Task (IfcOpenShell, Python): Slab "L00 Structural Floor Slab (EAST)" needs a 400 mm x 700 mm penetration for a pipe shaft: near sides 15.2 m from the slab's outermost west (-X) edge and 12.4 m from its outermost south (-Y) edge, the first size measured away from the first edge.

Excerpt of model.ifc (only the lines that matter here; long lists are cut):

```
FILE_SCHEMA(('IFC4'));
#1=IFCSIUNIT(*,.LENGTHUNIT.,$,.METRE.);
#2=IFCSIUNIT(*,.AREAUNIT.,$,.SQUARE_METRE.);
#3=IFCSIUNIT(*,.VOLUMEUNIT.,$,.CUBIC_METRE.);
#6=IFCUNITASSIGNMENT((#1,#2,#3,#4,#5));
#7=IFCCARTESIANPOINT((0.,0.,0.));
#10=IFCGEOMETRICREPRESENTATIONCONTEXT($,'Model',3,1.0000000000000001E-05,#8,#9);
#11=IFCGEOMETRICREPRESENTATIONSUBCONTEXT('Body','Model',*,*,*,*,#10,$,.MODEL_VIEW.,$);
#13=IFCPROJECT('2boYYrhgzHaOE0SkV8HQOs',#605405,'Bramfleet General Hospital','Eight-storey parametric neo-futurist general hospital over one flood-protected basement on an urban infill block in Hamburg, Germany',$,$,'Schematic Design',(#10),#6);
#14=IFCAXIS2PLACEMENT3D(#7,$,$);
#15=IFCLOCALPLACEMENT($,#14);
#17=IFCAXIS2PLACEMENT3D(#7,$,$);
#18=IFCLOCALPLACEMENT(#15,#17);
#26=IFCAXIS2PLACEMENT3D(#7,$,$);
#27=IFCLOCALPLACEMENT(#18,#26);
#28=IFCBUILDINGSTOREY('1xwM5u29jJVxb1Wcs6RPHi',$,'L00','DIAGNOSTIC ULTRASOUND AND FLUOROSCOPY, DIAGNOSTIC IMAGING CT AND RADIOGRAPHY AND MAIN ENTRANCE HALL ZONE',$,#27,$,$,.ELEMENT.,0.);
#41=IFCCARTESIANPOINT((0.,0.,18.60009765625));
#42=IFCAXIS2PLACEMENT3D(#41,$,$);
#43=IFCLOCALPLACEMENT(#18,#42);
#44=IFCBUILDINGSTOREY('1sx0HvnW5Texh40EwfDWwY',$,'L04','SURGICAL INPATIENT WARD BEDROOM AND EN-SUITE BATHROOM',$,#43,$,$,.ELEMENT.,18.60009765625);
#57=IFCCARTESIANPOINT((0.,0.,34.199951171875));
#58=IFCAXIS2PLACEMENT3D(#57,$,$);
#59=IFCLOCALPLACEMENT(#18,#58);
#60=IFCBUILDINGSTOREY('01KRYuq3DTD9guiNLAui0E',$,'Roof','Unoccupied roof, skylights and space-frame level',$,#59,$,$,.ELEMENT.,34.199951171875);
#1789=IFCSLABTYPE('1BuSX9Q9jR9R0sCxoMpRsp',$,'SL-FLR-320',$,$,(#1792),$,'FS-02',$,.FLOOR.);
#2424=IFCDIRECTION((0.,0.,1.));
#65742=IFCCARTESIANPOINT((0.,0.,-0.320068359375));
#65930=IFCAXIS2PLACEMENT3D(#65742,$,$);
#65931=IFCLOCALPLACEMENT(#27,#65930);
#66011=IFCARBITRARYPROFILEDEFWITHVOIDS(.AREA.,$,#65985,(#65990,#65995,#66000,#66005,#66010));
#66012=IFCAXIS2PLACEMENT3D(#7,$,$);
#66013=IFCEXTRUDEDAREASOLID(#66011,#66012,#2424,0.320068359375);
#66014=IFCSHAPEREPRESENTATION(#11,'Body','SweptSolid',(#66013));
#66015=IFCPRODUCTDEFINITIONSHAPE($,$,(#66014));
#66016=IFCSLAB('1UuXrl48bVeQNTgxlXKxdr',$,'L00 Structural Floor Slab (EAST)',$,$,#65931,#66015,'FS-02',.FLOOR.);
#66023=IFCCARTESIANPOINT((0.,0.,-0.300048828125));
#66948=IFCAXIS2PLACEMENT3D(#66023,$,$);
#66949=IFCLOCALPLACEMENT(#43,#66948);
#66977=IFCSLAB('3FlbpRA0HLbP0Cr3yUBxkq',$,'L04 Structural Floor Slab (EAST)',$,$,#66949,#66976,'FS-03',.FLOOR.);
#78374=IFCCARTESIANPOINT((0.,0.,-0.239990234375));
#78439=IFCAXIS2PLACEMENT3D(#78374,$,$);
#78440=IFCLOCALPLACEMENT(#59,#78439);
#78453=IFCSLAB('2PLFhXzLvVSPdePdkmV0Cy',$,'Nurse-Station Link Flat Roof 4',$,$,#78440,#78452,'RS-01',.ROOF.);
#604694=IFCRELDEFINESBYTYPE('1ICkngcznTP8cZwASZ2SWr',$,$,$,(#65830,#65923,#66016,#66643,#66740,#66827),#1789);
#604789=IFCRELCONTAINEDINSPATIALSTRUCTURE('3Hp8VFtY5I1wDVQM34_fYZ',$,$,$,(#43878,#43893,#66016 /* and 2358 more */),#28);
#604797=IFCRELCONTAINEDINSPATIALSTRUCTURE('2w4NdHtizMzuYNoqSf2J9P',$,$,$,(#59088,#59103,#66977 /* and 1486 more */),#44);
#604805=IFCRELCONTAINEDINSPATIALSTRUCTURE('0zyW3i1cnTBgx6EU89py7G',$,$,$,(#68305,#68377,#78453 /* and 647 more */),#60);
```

```python
import numpy as np
import ifcopenshell
import ifcopenshell.api.feature
import ifcopenshell.api.geometry
import ifcopenshell.api.root
import ifcopenshell.geom
import ifcopenshell.util.placement
import ifcopenshell.util.representation
import ifcopenshell.util.shape
import ifcopenshell.util.unit

model = ifcopenshell.open("model.ifc")
unit_scale = ifcopenshell.util.unit.calculate_unit_scale(model)
settings = ifcopenshell.geom.settings()


def volume(element):
    """Net volume in cubic metres, openings subtracted."""
    shape = ifcopenshell.geom.create_shape(settings, element)
    return ifcopenshell.util.shape.get_volume(shape.geometry)


slab = model.by_id(66016)
before = volume(slab)

# Extent in the slab's own axes, in metres. The edges named are its -X and -Y sides.
slab_shape = ifcopenshell.geom.create_shape(settings, slab)
vertices = ifcopenshell.util.shape.get_vertices(slab_shape.geometry)
x_min, y_min, bottom = vertices.min(axis=0)
top = vertices[:, 2].max()

opening = ifcopenshell.api.root.create_entity(model, ifc_class="IfcOpeningElement", name="Pipe shaft opening", predefined_type="OPENING")
context = ifcopenshell.util.representation.get_context(model, "Model", "Body", "MODEL_VIEW")
width, depth = 0.4, 0.7
outline = [(0.0, 0.0), (width, 0.0), (width, depth), (0.0, depth), (0.0, 0.0)]
# Overshoot both faces by 50 mm so the cut is clean.
shape = ifcopenshell.api.geometry.add_slab_representation(
    model, context=context, depth=top - bottom + 0.1, polyline=outline
)
ifcopenshell.api.geometry.assign_representation(model, product=opening, representation=shape)

matrix = ifcopenshell.util.placement.get_local_placement(slab.ObjectPlacement)
matrix[:, 3] = matrix @ np.append(np.array([x_min + 15.2, y_min + 12.4, bottom - 0.05]) / unit_scale, 1.0)
ifcopenshell.api.geometry.edit_object_placement(model, product=opening, matrix=matrix, is_si=False)
ifcopenshell.api.feature.add_feature(model, feature=opening, element=slab)

after = volume(slab)

print(f"slab volume {before:.3f} -> {after:.3f} m3")

model.write("model-out.ifc")
```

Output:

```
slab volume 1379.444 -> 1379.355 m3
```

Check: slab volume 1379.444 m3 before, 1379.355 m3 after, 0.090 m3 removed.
